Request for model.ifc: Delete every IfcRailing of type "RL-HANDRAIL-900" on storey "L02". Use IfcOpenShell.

First a look at what the model holds.

```python
import ifcopenshell
import ifcopenshell.util.element

model = ifcopenshell.open("model.ifc")
print(model.schema)
storey = next(s for s in model.by_type("IfcBuildingStorey") if s.Name == "L02")
railings = [e for e in ifcopenshell.util.element.get_decomposition(storey) if e.is_a("IfcRailing")]
seen = {}
for e in railings:
    element_type = ifcopenshell.util.element.get_type(e)
    name = element_type.Name if element_type not in (None, e) else None
    seen[name] = seen.get(name, 0) + 1
for name, count in sorted(seen.items(), key=str):
    print(count, "x", name)
```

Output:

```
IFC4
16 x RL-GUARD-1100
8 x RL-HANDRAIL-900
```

```python
import ifcopenshell
import ifcopenshell.api.root
import ifcopenshell.util.element

model = ifcopenshell.open("model.ifc")

storey = next(s for s in model.by_type("IfcBuildingStorey") if s.Name == "L02")
railings = [e for e in ifcopenshell.util.element.get_decomposition(storey) if e.is_a("IfcRailing")]
targets = [e for e in railings if (t := ifcopenshell.util.element.get_type(e)) not in (None, e) and t.Name == "RL-HANDRAIL-900"]

for e in targets:
    ifcopenshell.api.root.remove_product(model, product=e)
print(len(targets), "removed")

model.write("model_v2.ifc")
```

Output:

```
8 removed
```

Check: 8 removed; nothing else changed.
